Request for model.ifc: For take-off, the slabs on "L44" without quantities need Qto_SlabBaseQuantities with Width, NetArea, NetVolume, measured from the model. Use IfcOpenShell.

First a look at what the model holds.

```python
import ifcopenshell
import ifcopenshell.util.element
import ifcopenshell.util.unit

model = ifcopenshell.open("model.ifc")
print(model.schema)
for unit_type in ("LENGTHUNIT", "AREAUNIT", "VOLUMEUNIT"):
    print(unit_type, ifcopenshell.util.unit.calculate_unit_scale(model, unit_type))
storey = next(s for s in model.by_type("IfcBuildingStorey") if s.Name == "L44")
slabs = [e for e in ifcopenshell.util.element.get_decomposition(storey) if e.is_a("IfcSlab")]
for e in sorted(slabs, key=lambda e: e.id()):
    print(e.id(), e.is_a(), e.Name, list(ifcopenshell.util.element.get_psets(e, qtos_only=True)), sep=" | ")
```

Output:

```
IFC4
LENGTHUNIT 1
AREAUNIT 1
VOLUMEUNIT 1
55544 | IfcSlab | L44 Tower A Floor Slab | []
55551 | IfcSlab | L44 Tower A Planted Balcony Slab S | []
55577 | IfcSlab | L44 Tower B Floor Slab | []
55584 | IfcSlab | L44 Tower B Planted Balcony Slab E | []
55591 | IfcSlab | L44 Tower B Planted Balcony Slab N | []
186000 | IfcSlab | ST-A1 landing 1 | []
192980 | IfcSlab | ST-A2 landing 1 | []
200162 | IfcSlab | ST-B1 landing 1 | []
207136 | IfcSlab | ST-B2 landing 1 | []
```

```python
import ifcopenshell
import ifcopenshell.api.pset
import ifcopenshell.geom
import ifcopenshell.util.element
import ifcopenshell.util.shape
import ifcopenshell.util.unit

model = ifcopenshell.open("model.ifc")
unit_scale = ifcopenshell.util.unit.calculate_unit_scale(model)
area_scale = ifcopenshell.util.unit.calculate_unit_scale(model, "AREAUNIT")
volume_scale = ifcopenshell.util.unit.calculate_unit_scale(model, "VOLUMEUNIT")
settings = ifcopenshell.geom.settings()

storey = next(s for s in model.by_type("IfcBuildingStorey") if s.Name == "L44")
slabs = [e for e in ifcopenshell.util.element.get_decomposition(storey) if e.is_a("IfcSlab")]

for e in sorted(slabs, key=lambda e: e.id()):
    if ifcopenshell.util.element.get_psets(e, qtos_only=True, should_inherit=False):
        continue
    # Geometry comes back in metres, in the element's own axes.
    shape = ifcopenshell.geom.create_shape(settings, e)
    values = {
        "Width": ifcopenshell.util.shape.get_z(shape.geometry) / unit_scale,
        "NetArea": ifcopenshell.util.shape.get_footprint_area(shape.geometry) / area_scale,
        "NetVolume": ifcopenshell.util.shape.get_volume(shape.geometry) / volume_scale,
    }
    qto = ifcopenshell.api.pset.add_qto(model, product=e, name="Qto_SlabBaseQuantities")
    ifcopenshell.api.pset.edit_qto(model, qto=qto, properties=values)
    print(e.id(), {k: round(v, 3) for k, v in values.items()})

model.write("model_edited.ifc")
```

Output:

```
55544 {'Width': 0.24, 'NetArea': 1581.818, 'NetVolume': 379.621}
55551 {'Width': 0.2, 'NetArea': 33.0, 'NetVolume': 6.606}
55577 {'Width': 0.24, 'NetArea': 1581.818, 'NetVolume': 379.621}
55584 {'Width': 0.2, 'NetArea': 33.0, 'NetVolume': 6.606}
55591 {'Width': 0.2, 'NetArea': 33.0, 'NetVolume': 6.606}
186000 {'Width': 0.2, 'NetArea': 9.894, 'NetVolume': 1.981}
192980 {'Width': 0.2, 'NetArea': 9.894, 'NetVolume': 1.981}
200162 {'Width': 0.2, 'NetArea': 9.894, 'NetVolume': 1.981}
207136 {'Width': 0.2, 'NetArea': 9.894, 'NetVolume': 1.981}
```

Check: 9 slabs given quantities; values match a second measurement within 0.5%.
